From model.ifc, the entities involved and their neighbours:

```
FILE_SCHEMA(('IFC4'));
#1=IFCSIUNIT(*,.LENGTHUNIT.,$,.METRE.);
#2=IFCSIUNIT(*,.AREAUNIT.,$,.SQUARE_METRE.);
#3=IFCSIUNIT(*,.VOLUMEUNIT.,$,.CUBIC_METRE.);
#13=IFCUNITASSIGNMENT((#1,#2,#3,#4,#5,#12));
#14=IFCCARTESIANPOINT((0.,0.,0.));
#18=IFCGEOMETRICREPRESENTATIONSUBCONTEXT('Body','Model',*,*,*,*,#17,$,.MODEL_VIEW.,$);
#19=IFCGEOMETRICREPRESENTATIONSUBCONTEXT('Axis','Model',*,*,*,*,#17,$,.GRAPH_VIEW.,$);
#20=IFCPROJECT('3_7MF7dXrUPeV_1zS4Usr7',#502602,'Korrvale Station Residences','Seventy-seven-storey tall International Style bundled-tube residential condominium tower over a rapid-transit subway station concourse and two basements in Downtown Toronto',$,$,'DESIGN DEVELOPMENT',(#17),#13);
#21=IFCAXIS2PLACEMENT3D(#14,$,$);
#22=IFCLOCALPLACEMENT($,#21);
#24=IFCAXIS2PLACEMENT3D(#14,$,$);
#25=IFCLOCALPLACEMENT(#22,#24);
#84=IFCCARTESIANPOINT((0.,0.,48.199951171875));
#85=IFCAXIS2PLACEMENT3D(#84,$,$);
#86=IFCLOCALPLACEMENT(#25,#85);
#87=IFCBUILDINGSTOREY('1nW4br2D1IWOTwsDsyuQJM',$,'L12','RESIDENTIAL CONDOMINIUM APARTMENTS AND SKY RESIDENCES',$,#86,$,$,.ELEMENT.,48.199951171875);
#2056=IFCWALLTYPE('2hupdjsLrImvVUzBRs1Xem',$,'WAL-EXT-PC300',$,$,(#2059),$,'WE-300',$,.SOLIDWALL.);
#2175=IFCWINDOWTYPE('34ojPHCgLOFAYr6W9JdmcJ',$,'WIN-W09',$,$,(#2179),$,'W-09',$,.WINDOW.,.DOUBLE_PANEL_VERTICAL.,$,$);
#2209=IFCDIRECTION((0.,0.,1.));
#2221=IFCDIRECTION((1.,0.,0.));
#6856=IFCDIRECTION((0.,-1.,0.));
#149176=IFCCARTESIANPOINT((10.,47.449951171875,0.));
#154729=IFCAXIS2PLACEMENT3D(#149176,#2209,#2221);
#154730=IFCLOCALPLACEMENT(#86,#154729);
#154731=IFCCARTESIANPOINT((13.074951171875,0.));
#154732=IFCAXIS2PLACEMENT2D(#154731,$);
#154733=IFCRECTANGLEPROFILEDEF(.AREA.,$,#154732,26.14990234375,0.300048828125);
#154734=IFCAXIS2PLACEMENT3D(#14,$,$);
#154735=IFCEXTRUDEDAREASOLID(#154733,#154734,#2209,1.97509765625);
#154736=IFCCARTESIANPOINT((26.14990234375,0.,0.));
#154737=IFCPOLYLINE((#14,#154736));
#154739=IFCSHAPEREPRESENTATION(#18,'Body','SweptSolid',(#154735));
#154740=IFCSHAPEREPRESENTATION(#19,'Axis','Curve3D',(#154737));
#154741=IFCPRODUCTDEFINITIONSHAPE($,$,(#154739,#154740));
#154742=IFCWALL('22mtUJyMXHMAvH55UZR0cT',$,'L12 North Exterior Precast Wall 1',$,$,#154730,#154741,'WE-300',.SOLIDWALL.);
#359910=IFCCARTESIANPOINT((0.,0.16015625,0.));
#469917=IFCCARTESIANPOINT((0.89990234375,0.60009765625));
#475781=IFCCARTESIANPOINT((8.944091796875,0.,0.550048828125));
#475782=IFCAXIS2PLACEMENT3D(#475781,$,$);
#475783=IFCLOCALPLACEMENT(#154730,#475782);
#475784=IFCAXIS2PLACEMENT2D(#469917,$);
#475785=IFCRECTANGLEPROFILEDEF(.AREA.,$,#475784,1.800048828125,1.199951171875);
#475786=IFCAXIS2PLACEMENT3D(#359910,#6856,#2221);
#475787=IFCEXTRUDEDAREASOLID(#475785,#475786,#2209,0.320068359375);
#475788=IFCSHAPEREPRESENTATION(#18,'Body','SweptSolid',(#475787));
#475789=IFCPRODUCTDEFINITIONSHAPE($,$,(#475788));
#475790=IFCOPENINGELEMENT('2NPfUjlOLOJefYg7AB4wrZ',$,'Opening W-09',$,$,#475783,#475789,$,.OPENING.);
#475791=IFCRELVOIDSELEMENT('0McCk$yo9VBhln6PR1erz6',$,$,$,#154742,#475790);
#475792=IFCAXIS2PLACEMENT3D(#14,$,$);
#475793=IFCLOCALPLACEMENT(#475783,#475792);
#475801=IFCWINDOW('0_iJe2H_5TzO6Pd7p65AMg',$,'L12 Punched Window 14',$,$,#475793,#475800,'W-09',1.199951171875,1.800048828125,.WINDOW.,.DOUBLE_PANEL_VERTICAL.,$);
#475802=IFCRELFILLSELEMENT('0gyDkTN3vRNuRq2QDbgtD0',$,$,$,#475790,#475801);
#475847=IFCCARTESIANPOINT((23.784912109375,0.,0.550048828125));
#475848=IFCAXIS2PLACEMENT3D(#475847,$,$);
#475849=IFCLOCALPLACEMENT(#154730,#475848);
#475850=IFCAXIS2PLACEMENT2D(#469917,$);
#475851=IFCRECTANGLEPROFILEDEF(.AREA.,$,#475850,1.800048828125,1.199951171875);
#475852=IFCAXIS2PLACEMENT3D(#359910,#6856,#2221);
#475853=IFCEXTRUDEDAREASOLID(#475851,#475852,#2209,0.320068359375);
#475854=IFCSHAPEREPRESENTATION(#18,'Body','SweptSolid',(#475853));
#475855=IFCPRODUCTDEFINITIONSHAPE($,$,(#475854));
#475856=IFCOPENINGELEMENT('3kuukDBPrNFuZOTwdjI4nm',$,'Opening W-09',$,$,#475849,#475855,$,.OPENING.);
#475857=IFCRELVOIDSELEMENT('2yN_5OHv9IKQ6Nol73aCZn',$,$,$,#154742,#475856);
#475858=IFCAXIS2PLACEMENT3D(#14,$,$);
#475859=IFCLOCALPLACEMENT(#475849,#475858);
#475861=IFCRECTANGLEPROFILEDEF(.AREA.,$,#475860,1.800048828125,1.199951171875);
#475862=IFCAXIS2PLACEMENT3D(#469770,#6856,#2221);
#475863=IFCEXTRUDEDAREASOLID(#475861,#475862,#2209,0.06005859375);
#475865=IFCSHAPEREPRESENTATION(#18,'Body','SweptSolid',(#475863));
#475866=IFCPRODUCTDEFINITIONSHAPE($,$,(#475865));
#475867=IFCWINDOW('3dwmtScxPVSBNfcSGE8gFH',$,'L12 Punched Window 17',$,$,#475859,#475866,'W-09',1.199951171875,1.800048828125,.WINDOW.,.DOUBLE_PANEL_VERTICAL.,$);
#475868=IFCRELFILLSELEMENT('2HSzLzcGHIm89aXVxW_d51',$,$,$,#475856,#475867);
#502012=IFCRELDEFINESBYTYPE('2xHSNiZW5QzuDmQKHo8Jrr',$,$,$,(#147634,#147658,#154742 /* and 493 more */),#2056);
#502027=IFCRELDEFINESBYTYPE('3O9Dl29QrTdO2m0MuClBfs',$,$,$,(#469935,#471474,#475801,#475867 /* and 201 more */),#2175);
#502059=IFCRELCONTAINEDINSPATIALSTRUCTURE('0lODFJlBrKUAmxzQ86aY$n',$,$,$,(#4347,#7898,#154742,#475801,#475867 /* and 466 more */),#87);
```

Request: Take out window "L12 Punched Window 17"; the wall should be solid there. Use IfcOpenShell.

```python
import ifcopenshell
import ifcopenshell.api.feature
import ifcopenshell.api.root
import ifcopenshell.geom
import ifcopenshell.util.shape

model = ifcopenshell.open("model.ifc")
settings = ifcopenshell.geom.settings()


def volume(element):
    """Net volume in cubic metres, openings subtracted."""
    shape = ifcopenshell.geom.create_shape(settings, element)
    return ifcopenshell.util.shape.get_volume(shape.geometry)


window = model.by_guid("3dwmtScxPVSBNfcSGE8gFH")
opening = window.FillsVoids[0].RelatingOpeningElement
wall = opening.VoidsElements[0].RelatingBuildingElement
before = volume(wall)

ifcopenshell.api.root.remove_product(model, product=window)
ifcopenshell.api.feature.remove_feature(model, feature=opening)

after = volume(wall)

print(f"wall volume {before:.3f} -> {after:.3f} m3")

model.write("model_rev.ifc")
```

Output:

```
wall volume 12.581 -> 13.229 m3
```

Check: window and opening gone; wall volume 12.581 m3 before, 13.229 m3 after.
